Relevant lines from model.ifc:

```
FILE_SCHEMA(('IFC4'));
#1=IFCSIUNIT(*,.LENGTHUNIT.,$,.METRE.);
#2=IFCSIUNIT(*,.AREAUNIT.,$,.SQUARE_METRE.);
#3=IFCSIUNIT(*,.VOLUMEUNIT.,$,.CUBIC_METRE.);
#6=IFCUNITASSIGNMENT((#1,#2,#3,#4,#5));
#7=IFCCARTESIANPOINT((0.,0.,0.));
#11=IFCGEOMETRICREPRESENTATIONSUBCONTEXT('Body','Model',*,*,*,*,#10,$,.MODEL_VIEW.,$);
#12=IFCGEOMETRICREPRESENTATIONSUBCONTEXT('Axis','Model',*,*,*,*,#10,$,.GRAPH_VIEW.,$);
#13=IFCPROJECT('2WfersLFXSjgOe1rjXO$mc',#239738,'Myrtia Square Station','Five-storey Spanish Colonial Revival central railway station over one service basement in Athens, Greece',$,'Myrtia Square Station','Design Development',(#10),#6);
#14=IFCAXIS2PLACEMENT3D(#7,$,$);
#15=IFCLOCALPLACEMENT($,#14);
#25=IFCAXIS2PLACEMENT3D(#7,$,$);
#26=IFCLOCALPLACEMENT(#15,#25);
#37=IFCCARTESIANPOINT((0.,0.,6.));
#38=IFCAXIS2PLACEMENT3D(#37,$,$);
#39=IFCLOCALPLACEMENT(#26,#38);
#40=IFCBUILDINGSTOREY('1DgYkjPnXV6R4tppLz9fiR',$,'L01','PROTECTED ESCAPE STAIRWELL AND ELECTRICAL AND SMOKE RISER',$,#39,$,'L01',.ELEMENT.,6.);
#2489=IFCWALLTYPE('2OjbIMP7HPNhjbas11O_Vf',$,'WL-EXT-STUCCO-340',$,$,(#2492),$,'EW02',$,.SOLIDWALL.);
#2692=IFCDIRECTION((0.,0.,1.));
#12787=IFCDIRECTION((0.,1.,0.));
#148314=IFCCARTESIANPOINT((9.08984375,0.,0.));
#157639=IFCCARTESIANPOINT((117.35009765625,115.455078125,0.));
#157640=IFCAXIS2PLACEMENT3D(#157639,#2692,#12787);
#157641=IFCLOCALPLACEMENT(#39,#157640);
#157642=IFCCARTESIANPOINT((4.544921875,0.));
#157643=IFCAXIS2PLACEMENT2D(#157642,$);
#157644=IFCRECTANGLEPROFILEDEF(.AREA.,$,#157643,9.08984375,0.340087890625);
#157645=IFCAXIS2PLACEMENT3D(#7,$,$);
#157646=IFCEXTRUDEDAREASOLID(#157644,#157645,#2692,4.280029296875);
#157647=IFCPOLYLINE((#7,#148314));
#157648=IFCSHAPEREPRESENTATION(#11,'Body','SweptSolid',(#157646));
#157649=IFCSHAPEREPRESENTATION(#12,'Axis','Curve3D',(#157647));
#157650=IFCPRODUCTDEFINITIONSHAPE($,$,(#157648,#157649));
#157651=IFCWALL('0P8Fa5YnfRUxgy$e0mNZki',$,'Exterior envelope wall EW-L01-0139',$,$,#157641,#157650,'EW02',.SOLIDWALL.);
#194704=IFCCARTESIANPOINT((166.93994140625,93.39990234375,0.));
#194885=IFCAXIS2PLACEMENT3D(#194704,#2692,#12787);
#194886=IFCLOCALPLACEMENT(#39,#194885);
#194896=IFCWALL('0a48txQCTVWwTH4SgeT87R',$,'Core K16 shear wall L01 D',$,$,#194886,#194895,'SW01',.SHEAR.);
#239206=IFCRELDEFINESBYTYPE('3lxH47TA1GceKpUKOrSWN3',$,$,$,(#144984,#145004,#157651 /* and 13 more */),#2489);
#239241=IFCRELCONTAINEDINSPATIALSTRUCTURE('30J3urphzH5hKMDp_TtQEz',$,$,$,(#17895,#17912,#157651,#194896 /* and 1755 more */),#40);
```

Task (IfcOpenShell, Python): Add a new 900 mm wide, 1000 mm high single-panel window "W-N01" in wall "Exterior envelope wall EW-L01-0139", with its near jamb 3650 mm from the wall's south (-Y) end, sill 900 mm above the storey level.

```python
import numpy as np
import ifcopenshell
import ifcopenshell.api.feature
import ifcopenshell.api.geometry
import ifcopenshell.api.root
import ifcopenshell.api.spatial
import ifcopenshell.geom
import ifcopenshell.util.element
import ifcopenshell.util.placement
import ifcopenshell.util.representation
import ifcopenshell.util.shape
import ifcopenshell.util.unit

model = ifcopenshell.open("model.ifc")
unit_scale = ifcopenshell.util.unit.calculate_unit_scale(model)
settings = ifcopenshell.geom.settings()


def volume(element):
    """Net volume in cubic metres, openings subtracted."""
    shape = ifcopenshell.geom.create_shape(settings, element)
    return ifcopenshell.util.shape.get_volume(shape.geometry)


wall = model.by_guid("0P8Fa5YnfRUxgy$e0mNZki")
storey = ifcopenshell.util.element.get_container(wall, ifc_class="IfcBuildingStorey")
context = ifcopenshell.util.representation.get_context(model, "Model", "Body", "MODEL_VIEW")
before = volume(wall)

width, height, from_end, sill = 0.9, 1, 3.65, 0.9  # metres

# The wall runs along its own X axis, and the end named is its -X end.
wall_shape = ifcopenshell.geom.create_shape(settings, wall)
x, y, z = ifcopenshell.util.shape.get_vertices(wall_shape.geometry).T
start = x.min() + from_end
face, thickness = float(y.min()), float(y.max() - y.min())
wall_matrix = ifcopenshell.util.placement.get_local_placement(wall.ObjectPlacement)
level = ifcopenshell.util.placement.get_local_placement(storey.ObjectPlacement)[2, 3]


def in_wall(x, y):
    """Placement at x, y metres in the wall's axes, at sill height."""
    matrix = wall_matrix.copy()
    matrix[:, 3] = wall_matrix @ np.array([x / unit_scale, y / unit_scale, 0.0, 1.0])
    matrix[2, 3] = level + sill / unit_scale
    return matrix


# Opening: a box that overshoots both wall faces by 50 mm.
opening = ifcopenshell.api.root.create_entity(model, ifc_class="IfcOpeningElement", predefined_type="OPENING")
box = ifcopenshell.api.geometry.add_wall_representation(
    model, context=context, length=width, height=height, thickness=thickness + 0.1
)
ifcopenshell.api.geometry.assign_representation(model, product=opening, representation=box)
ifcopenshell.api.geometry.edit_object_placement(model, product=opening, matrix=in_wall(start, face - 0.05), is_si=False)
ifcopenshell.api.feature.add_feature(model, feature=opening, element=wall)

window = ifcopenshell.api.root.create_entity(model, ifc_class="IfcWindow", name="W-N01", predefined_type="WINDOW")
window.OverallWidth, window.OverallHeight = width / unit_scale, height / unit_scale
window.PartitioningType = "SINGLE_PANEL"
body = ifcopenshell.api.geometry.add_window_representation(
    model,
    context=context,
    overall_width=window.OverallWidth,
    overall_height=window.OverallHeight,
    partition_type="SINGLE_PANEL",
)
ifcopenshell.api.geometry.assign_representation(model, product=window, representation=body)
ifcopenshell.api.spatial.assign_container(model, products=[window], relating_structure=storey)
ifcopenshell.api.feature.add_filling(model, opening=opening, element=window)

# Centre the window in the wall's thickness.
ifcopenshell.api.geometry.edit_object_placement(model, product=window, matrix=in_wall(start, face), is_si=False)
window_shape = ifcopenshell.geom.create_shape(settings, window)
depth = ifcopenshell.util.shape.get_vertices(window_shape.geometry)[:, 1]
offset = face + thickness / 2 - (depth.min() + depth.max()) / 2
ifcopenshell.api.geometry.edit_object_placement(model, product=window, matrix=in_wall(start, offset), is_si=False)

after = volume(wall)

print(f"wall volume {before:.3f} -> {after:.3f} m3")

model.write("model_v2.ifc")
```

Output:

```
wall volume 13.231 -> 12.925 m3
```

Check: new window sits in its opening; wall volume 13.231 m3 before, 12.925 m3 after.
